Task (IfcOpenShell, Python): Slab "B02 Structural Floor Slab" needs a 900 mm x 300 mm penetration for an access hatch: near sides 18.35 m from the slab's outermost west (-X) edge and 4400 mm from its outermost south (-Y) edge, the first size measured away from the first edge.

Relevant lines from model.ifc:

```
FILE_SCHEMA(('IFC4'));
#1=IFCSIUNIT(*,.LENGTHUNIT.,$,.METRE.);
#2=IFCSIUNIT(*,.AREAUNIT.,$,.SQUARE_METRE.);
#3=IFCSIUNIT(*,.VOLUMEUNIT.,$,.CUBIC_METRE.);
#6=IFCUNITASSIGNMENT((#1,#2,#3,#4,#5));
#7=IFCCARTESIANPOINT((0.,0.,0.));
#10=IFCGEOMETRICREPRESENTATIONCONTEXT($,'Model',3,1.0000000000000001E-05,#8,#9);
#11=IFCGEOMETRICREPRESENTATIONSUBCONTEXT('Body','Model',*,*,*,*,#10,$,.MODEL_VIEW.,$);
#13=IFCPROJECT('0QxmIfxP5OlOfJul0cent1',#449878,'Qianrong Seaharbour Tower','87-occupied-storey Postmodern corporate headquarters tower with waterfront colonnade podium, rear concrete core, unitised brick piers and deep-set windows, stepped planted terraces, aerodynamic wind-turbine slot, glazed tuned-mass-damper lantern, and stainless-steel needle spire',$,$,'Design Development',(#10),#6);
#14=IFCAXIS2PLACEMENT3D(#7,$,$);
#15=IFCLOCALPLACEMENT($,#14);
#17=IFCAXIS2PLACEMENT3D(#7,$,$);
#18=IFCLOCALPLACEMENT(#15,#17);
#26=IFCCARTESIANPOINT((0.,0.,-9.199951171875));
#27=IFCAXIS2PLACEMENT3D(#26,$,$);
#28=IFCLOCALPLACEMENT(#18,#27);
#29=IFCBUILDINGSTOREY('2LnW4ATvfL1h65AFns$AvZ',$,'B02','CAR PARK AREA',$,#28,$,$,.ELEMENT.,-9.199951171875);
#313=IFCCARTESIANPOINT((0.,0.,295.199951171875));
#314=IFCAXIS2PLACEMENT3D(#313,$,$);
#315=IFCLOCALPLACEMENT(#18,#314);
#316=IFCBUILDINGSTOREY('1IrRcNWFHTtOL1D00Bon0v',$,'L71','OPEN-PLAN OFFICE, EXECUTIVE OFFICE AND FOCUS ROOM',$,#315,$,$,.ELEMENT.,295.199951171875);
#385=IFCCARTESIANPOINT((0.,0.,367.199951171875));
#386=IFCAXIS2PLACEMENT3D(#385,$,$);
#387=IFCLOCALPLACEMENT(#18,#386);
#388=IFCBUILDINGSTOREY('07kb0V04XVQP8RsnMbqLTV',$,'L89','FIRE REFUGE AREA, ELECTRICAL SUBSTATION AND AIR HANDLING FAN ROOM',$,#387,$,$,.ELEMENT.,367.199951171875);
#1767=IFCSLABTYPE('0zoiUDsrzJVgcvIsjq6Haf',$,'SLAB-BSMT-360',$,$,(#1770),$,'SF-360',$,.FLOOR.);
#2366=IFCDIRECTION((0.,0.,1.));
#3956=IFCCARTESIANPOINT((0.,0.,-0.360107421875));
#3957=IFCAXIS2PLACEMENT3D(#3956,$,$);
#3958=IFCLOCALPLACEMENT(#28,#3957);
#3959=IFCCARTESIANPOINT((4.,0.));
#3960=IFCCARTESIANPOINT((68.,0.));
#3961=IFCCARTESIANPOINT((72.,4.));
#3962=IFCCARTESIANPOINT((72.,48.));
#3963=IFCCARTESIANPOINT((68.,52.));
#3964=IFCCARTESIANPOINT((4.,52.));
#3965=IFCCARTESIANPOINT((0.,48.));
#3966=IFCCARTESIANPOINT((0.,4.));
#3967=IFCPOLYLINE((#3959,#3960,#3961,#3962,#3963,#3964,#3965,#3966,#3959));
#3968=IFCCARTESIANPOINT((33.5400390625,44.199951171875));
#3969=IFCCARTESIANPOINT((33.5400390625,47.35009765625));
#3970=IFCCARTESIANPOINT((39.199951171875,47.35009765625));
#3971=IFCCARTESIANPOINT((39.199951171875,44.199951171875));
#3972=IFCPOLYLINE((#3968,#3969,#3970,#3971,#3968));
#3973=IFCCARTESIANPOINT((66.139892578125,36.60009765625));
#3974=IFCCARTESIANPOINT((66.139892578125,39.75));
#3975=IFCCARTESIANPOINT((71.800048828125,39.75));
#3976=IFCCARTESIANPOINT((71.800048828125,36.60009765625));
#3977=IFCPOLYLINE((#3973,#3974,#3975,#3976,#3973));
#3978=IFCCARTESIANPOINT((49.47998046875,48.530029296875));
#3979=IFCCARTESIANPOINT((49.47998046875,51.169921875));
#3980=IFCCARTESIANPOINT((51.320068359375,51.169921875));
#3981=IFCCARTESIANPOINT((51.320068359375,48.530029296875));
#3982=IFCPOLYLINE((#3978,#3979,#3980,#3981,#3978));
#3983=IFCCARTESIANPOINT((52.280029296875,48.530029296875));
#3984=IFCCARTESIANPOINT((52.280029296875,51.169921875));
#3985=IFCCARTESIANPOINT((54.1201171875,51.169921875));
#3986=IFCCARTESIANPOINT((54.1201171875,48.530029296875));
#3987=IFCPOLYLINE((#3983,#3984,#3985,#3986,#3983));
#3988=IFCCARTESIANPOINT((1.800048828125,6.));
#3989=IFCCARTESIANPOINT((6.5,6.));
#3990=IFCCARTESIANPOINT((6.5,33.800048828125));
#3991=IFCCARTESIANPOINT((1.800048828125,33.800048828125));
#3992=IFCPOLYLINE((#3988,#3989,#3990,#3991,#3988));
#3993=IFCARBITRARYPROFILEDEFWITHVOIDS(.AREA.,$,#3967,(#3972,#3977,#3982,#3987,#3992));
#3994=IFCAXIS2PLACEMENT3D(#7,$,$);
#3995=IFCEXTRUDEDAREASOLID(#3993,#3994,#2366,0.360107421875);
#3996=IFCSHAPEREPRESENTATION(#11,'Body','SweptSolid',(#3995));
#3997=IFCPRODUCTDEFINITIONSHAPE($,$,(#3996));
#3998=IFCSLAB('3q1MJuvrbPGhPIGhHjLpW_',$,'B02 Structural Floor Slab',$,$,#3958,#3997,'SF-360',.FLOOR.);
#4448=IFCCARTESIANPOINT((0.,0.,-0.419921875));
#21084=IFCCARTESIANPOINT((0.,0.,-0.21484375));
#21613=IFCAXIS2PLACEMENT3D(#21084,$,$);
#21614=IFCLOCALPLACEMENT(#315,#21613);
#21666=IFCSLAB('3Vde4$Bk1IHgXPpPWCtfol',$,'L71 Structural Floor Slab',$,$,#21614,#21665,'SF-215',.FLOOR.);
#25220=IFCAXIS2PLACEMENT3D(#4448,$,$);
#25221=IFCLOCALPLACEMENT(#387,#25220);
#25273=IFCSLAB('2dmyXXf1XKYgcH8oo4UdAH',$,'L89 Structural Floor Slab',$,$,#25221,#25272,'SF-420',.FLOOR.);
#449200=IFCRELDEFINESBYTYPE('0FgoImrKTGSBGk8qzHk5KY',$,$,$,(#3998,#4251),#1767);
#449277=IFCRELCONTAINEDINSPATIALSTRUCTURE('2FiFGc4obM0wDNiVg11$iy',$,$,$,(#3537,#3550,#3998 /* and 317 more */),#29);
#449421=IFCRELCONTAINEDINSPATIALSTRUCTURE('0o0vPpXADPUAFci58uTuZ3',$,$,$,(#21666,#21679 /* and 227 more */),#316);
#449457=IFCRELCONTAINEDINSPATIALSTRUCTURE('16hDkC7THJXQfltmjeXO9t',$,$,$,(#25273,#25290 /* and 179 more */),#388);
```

```python
import numpy as np
import ifcopenshell
import ifcopenshell.api.feature
import ifcopenshell.api.geometry
import ifcopenshell.api.root
import ifcopenshell.geom
import ifcopenshell.util.placement
import ifcopenshell.util.representation
import ifcopenshell.util.shape
import ifcopenshell.util.unit

model = ifcopenshell.open("model.ifc")
unit_scale = ifcopenshell.util.unit.calculate_unit_scale(model)
settings = ifcopenshell.geom.settings()


def volume(element):
    """Net volume in cubic metres, openings subtracted."""
    shape = ifcopenshell.geom.create_shape(settings, element)
    return ifcopenshell.util.shape.get_volume(shape.geometry)


slab = model.by_guid("3q1MJuvrbPGhPIGhHjLpW_")
before = volume(slab)

# Extent in the slab's own axes, in metres. The edges named are its -X and -Y sides.
slab_shape = ifcopenshell.geom.create_shape(settings, slab)
vertices = ifcopenshell.util.shape.get_vertices(slab_shape.geometry)
x_min, y_min, bottom = vertices.min(axis=0)
top = vertices[:, 2].max()

opening = ifcopenshell.api.root.create_entity(model, ifc_class="IfcOpeningElement", name="Access hatch opening", predefined_type="OPENING")
context = ifcopenshell.util.representation.get_context(model, "Model", "Body", "MODEL_VIEW")
width, depth = 0.9, 0.3
outline = [(0.0, 0.0), (width, 0.0), (width, depth), (0.0, depth), (0.0, 0.0)]
# Overshoot both faces by 50 mm so the cut is clean.
shape = ifcopenshell.api.geometry.add_slab_representation(
    model, context=context, depth=top - bottom + 0.1, polyline=outline
)
ifcopenshell.api.geometry.assign_representation(model, product=opening, representation=shape)

matrix = ifcopenshell.util.placement.get_local_placement(slab.ObjectPlacement)
matrix[:, 3] = matrix @ np.append(np.array([x_min + 18.35, y_min + 4.4, bottom - 0.05]) / unit_scale, 1.0)
ifcopenshell.api.geometry.edit_object_placement(model, product=opening, matrix=matrix, is_si=False)
ifcopenshell.api.feature.add_feature(model, feature=opening, element=slab)

after = volume(slab)

print(f"slab volume {before:.3f} -> {after:.3f} m3")

model.write("model-out.ifc")
```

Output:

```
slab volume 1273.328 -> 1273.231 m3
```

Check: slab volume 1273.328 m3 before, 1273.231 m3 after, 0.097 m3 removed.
